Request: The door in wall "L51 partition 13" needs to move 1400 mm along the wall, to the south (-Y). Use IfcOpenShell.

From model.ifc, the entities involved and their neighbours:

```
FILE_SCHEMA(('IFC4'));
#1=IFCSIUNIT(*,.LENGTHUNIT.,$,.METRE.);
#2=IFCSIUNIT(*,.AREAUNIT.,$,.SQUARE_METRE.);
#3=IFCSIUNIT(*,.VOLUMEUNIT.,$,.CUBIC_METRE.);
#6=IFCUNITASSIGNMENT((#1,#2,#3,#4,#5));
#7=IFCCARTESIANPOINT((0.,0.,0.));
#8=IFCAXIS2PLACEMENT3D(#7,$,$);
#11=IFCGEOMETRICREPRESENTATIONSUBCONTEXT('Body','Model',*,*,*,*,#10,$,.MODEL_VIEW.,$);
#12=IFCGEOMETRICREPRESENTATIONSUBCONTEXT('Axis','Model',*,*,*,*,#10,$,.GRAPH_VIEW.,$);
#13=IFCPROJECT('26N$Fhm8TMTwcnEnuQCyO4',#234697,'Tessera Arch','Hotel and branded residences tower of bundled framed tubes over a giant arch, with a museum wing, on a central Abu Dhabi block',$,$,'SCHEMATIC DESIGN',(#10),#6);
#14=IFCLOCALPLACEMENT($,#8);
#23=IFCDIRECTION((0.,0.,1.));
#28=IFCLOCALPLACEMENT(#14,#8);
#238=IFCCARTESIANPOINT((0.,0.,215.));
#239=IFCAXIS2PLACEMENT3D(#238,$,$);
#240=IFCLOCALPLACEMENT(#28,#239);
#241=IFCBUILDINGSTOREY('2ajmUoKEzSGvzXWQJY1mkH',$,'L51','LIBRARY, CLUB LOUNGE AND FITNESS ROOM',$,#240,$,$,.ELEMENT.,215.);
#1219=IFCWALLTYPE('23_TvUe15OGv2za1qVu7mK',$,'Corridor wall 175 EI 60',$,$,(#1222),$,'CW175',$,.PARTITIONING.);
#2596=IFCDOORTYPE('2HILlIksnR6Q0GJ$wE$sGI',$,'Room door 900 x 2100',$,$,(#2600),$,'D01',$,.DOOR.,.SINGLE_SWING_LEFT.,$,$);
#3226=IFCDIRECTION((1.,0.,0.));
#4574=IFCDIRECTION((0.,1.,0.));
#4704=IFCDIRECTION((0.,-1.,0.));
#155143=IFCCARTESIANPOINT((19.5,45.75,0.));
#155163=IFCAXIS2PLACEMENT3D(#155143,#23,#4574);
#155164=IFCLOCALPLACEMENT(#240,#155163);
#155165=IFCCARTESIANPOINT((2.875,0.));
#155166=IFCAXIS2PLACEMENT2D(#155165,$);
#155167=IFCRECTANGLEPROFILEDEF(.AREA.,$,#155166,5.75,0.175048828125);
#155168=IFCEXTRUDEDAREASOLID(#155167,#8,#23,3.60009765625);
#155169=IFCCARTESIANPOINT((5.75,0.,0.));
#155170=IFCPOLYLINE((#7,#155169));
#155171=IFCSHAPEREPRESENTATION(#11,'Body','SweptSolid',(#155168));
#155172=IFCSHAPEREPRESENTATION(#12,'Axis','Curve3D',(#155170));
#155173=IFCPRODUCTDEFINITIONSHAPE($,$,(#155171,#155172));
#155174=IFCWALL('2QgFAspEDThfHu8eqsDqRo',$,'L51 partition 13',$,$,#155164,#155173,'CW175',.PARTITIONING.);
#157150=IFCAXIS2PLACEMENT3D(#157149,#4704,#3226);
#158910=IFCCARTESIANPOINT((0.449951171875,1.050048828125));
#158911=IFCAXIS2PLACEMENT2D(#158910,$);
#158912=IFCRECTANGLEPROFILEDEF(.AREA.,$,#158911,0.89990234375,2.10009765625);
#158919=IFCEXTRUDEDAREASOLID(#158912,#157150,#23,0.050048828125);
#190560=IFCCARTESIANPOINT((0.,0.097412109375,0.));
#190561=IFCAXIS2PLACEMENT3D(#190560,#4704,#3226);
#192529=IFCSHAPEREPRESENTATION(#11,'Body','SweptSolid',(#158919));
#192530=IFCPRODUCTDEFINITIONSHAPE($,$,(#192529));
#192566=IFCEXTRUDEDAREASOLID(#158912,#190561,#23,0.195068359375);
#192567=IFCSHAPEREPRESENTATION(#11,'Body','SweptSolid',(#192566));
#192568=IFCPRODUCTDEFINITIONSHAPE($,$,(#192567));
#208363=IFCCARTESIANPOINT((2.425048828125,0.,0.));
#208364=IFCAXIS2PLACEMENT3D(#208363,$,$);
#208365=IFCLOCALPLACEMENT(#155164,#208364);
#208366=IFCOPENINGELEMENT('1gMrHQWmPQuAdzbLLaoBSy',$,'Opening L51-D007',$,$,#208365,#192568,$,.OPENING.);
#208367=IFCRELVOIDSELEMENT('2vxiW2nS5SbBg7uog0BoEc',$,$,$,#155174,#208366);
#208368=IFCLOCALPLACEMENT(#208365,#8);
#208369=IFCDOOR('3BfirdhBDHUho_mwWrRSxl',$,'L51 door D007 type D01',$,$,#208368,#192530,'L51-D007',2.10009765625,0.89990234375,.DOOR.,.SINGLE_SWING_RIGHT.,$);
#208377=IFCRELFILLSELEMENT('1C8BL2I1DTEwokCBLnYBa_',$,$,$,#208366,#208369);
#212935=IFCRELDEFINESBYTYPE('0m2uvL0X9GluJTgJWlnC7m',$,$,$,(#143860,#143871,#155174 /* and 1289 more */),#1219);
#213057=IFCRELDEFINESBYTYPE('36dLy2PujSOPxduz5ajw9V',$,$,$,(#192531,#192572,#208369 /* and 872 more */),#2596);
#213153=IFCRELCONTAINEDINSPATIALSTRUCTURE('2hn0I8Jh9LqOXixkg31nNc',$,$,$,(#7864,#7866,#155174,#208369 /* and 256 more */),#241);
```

```python
import ifcopenshell
import ifcopenshell.api.geometry
import ifcopenshell.util.placement
import ifcopenshell.util.unit

model = ifcopenshell.open("model.ifc")
unit_scale = ifcopenshell.util.unit.calculate_unit_scale(model)

door = model.by_guid("3BfirdhBDHUho_mwWrRSxl")
opening = door.FillsVoids[0].RelatingOpeningElement
wall = opening.VoidsElements[0].RelatingBuildingElement

wall_matrix = ifcopenshell.util.placement.get_local_placement(wall.ObjectPlacement)
shift = wall_matrix[:3, 0] * -1.4 / unit_scale
before = ifcopenshell.util.placement.get_local_placement(door.ObjectPlacement)[:3, 3].copy()

# The door is placed relative to its opening, so it follows when the opening moves.
matrix = ifcopenshell.util.placement.get_local_placement(opening.ObjectPlacement)
matrix[:3, 3] += shift
ifcopenshell.api.geometry.edit_object_placement(
    model, product=opening, matrix=matrix, is_si=False, should_transform_children=True
)

after = ifcopenshell.util.placement.get_local_placement(door.ObjectPlacement)[:3, 3]
print("door moved by", (after - before).round(3) + 0.0)

model.write("model_rev.ifc")
```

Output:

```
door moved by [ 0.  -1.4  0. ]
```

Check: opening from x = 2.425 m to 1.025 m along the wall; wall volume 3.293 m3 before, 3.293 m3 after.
